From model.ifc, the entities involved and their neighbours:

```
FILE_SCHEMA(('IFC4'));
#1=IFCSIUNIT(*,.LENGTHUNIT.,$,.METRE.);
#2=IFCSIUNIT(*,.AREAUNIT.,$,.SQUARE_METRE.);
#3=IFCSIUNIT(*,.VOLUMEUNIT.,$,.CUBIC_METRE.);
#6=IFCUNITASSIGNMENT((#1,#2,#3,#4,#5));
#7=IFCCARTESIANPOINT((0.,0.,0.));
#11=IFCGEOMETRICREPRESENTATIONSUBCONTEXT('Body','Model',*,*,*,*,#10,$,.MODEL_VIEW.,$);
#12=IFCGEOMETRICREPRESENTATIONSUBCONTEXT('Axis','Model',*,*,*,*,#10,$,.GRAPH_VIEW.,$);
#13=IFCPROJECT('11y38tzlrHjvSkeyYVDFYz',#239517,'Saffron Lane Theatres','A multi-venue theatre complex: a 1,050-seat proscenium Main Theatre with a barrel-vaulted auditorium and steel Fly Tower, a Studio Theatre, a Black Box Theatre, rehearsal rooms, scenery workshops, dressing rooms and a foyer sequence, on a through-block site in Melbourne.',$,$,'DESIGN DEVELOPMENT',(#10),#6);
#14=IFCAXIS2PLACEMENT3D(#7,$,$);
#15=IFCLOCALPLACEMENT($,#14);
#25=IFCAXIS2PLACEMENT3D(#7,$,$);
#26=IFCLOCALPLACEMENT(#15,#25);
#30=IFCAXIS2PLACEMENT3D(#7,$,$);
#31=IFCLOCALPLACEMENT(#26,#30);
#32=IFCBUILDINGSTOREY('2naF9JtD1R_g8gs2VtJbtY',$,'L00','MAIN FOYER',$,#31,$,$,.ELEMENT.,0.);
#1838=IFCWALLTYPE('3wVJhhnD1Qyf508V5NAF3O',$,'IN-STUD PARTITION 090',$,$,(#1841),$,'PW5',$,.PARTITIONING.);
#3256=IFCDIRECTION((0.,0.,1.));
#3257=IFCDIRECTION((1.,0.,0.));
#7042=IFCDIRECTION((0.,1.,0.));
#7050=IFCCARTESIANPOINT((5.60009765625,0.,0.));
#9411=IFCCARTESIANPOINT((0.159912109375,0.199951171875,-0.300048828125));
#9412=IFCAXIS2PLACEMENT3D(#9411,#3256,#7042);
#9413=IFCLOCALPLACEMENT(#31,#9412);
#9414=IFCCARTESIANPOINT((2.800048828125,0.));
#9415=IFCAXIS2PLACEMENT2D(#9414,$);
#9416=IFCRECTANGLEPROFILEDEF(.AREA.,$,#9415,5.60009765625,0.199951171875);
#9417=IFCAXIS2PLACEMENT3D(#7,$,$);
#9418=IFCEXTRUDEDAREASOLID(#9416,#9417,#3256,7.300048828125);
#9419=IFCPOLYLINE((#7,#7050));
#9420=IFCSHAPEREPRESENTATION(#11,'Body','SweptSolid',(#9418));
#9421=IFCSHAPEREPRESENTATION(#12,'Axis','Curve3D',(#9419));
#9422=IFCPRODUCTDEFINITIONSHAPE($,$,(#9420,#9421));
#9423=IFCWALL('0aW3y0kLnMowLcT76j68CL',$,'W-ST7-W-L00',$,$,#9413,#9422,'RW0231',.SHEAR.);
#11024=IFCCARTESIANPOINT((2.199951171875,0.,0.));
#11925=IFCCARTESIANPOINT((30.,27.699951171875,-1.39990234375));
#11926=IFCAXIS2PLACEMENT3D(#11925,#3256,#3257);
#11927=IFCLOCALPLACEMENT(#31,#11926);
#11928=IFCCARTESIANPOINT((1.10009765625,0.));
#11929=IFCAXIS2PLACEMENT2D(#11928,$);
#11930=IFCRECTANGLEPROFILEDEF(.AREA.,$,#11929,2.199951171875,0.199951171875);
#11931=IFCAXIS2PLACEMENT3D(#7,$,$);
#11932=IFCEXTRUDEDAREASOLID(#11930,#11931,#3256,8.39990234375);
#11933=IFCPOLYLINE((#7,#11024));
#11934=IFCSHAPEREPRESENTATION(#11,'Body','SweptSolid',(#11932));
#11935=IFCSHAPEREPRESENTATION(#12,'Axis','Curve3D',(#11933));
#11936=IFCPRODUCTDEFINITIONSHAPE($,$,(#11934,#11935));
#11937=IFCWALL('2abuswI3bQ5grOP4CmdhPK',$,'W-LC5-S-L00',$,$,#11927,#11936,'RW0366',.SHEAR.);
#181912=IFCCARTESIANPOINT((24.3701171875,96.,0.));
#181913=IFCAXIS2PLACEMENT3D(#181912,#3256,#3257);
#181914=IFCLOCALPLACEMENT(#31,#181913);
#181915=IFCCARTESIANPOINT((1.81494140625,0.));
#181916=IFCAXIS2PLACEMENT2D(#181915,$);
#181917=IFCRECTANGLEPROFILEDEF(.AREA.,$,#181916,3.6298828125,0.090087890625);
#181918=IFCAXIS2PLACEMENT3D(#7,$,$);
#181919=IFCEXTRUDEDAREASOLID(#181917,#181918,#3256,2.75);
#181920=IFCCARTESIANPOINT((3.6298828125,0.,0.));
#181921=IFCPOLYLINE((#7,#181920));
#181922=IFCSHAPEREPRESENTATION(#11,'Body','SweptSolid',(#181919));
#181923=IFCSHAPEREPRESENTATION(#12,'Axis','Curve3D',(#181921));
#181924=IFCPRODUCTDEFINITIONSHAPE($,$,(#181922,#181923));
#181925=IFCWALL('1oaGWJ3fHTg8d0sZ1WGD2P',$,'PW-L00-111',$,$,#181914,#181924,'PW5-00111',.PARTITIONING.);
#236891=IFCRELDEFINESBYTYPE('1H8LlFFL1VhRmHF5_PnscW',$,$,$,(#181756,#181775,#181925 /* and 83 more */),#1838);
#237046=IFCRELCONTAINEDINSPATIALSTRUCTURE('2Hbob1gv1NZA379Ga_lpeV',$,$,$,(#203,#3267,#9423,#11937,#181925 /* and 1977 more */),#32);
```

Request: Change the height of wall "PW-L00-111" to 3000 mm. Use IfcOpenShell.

```python
import ifcopenshell
import ifcopenshell.geom
import ifcopenshell.util.representation
import ifcopenshell.util.shape

model = ifcopenshell.open("model.ifc")
settings = ifcopenshell.geom.settings()


def volume(element):
    """Net volume in cubic metres, openings subtracted."""
    shape = ifcopenshell.geom.create_shape(settings, element)
    return ifcopenshell.util.shape.get_volume(shape.geometry)


wall = model.by_guid("1oaGWJ3fHTg8d0sZ1WGD2P")
before = volume(wall)

body = ifcopenshell.util.representation.get_representation(wall, "Model", "Body")
solid = body.Items[0]
old_height = solid.Depth
solid.Depth = 3.0
after = volume(wall)

print(f"height {old_height:g} -> {solid.Depth:g}, volume {before:.3f} -> {after:.3f} m3")

model.write("model_updated.ifc")
```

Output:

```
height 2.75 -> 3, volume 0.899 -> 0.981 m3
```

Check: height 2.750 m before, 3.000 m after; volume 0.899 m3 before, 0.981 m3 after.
